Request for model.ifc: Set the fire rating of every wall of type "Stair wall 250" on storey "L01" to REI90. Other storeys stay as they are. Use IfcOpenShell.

First a look at what the model holds.

```python
import ifcopenshell
import ifcopenshell.util.element

model = ifcopenshell.open("model.ifc")
print(model.schema)
storey = next(s for s in model.by_type("IfcBuildingStorey") if s.Name == "L01")
walls = [e for e in ifcopenshell.util.element.get_decomposition(storey) if e.is_a("IfcWall")]
seen = {}
for e in walls:
    element_type = ifcopenshell.util.element.get_type(e)
    key = (element_type.Name if element_type != e and element_type else None, ifcopenshell.util.element.get_pset(e, "Pset_WallCommon", "FireRating"))
    seen[key] = seen.get(key, 0) + 1
for (name, value), count in sorted(seen.items(), key=str):
    print(count, "x", name, "|", value)
```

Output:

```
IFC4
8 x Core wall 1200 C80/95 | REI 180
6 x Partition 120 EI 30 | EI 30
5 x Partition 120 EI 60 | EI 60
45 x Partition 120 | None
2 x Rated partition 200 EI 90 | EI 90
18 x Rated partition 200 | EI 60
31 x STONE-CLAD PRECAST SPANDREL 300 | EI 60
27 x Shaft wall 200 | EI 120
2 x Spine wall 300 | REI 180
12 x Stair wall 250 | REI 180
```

```python
import ifcopenshell
import ifcopenshell.api.pset
import ifcopenshell.util.element

model = ifcopenshell.open("model.ifc")

storey = next(s for s in model.by_type("IfcBuildingStorey") if s.Name == "L01")
walls = [e for e in ifcopenshell.util.element.get_decomposition(storey) if e.is_a("IfcWall")]

count = 0
for e in walls:
    element_type = ifcopenshell.util.element.get_type(e)
    if element_type in (None, e) or element_type.Name != "Stair wall 250":
        continue
    found = ifcopenshell.util.element.get_pset(e, "Pset_WallCommon", should_inherit=False)
    if found:
        pset = model.by_id(found["id"])
        if len(ifcopenshell.util.element.get_elements_by_pset(pset)) > 1:
            pset = ifcopenshell.api.pset.unshare_pset(model, products=[e], pset=pset)[0]
    else:
        pset = ifcopenshell.api.pset.add_pset(model, product=e, name="Pset_WallCommon")
    ifcopenshell.api.pset.edit_pset(model, pset=pset, properties={"FireRating": "REI90"})
    count += 1

print(count, "walls updated")

model.write("model_v2.ifc")
```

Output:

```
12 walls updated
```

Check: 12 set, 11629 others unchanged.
